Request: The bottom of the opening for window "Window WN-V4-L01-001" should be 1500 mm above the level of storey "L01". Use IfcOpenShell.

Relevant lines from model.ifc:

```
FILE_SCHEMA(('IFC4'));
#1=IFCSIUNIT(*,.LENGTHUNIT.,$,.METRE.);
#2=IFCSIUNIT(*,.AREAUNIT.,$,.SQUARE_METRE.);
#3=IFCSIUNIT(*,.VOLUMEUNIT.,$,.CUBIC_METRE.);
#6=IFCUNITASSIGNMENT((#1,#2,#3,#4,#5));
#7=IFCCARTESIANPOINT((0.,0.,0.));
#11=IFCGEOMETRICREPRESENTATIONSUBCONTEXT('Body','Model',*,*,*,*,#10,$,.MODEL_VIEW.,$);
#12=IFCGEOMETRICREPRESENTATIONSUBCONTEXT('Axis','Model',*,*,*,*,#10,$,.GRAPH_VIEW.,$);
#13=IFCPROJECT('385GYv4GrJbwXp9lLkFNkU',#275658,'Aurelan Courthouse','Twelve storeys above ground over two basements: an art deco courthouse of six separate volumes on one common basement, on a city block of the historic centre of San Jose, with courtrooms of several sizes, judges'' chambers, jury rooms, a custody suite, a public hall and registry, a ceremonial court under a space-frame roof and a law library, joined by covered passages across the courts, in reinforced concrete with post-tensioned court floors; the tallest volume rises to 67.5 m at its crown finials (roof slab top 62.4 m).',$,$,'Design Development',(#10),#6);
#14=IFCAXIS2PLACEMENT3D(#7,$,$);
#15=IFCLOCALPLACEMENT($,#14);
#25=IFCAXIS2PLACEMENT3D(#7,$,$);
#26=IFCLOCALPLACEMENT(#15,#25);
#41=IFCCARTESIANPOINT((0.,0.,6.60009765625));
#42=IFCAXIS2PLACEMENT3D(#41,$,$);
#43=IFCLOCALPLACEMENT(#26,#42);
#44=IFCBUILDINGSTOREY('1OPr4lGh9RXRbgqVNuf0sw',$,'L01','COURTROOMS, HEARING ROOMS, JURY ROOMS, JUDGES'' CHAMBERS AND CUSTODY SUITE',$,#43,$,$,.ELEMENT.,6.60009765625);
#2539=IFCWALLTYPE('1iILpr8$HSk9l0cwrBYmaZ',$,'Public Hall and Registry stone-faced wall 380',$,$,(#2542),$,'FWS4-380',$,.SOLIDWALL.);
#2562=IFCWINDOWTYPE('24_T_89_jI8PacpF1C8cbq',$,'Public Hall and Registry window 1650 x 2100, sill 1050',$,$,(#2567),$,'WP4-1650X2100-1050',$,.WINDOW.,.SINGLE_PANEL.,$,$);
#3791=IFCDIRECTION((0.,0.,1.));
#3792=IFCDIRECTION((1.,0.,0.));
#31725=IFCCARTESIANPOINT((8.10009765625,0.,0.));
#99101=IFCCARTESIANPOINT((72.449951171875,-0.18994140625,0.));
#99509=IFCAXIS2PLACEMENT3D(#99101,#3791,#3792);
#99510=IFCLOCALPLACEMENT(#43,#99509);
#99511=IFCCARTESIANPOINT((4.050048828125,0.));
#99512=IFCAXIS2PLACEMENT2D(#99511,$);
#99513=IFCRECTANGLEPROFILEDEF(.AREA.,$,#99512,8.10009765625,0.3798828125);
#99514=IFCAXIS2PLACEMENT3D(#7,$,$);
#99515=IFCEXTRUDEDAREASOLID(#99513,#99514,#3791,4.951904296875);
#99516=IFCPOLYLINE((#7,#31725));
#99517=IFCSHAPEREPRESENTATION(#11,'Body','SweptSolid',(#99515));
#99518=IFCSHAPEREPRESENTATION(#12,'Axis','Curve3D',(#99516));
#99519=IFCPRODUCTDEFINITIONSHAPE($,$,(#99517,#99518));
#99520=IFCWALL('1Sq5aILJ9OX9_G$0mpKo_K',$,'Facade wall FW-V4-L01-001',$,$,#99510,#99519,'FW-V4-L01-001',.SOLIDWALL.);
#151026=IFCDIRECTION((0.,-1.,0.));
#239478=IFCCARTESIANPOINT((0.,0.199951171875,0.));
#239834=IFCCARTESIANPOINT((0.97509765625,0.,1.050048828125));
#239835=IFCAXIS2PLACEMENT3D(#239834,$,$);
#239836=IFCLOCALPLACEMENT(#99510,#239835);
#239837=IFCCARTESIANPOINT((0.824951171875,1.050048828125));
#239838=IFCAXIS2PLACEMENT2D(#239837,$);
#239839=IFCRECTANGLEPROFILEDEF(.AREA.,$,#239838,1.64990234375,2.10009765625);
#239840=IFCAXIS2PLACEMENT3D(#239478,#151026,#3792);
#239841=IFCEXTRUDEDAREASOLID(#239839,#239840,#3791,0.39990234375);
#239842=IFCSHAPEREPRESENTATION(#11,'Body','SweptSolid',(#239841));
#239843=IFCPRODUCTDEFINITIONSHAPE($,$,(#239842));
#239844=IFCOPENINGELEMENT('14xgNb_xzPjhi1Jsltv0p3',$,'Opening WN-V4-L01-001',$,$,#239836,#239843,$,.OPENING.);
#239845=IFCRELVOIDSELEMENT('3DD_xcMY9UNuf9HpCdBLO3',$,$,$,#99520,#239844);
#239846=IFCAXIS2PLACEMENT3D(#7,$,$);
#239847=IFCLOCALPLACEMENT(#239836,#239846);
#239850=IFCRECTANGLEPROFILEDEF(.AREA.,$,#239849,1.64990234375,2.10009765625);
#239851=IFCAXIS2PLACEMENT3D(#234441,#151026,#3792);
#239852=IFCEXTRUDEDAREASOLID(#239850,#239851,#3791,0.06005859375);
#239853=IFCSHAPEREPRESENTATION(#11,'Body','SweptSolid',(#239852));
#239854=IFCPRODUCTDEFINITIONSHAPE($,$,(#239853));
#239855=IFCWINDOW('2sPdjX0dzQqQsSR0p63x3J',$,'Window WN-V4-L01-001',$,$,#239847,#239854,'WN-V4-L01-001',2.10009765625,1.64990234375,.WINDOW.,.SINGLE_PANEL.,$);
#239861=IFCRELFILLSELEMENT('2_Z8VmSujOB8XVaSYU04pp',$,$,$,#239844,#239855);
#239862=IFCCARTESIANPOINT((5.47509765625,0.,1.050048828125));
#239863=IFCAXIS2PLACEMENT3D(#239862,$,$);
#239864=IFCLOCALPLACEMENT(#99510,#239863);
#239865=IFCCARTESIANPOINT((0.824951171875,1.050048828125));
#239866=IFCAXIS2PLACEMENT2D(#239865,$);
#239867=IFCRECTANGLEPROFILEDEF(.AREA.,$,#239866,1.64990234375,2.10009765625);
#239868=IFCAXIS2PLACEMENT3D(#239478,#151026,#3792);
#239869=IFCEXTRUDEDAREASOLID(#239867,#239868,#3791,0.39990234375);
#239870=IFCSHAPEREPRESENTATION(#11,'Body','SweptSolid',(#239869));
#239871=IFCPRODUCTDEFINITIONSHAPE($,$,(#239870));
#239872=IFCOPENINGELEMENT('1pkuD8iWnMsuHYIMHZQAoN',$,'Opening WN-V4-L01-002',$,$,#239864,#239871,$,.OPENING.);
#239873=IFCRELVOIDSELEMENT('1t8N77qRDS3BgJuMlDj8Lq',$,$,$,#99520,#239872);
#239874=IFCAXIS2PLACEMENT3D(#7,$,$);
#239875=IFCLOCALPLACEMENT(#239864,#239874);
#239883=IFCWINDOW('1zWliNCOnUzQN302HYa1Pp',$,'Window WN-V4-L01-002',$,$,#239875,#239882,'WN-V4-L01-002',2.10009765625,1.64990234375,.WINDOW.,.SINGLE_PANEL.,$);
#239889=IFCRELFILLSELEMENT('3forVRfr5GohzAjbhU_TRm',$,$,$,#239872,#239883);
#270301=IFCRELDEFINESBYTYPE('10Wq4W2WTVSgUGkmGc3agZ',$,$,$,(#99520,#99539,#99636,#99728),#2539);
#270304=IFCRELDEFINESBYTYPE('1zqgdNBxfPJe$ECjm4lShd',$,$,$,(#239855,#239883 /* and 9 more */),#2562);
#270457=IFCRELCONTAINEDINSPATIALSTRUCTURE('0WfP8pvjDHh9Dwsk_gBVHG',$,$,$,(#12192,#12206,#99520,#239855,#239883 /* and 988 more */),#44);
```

```python
import numpy as np
import ifcopenshell
import ifcopenshell.api.geometry
import ifcopenshell.geom
import ifcopenshell.util.element
import ifcopenshell.util.placement
import ifcopenshell.util.shape
import ifcopenshell.util.unit

model = ifcopenshell.open("model.ifc")
unit_scale = ifcopenshell.util.unit.calculate_unit_scale(model)

window = model.by_guid("2sPdjX0dzQqQsSR0p63x3J")
opening = window.FillsVoids[0].RelatingOpeningElement
storey = ifcopenshell.util.element.get_container(window, ifc_class="IfcBuildingStorey")
level = ifcopenshell.util.placement.get_local_placement(storey.ObjectPlacement)[2, 3]

# The opening's origin need not be at the sill, so measure its lowest point.
shape = ifcopenshell.geom.create_shape(ifcopenshell.geom.settings(), opening)
bottom = ifcopenshell.util.shape.get_shape_bottom_elevation(shape, shape.geometry) / unit_scale
dz = level + 1.5 - bottom

shift = np.array([0.0, 0.0, dz])
# The window is placed relative to its opening, so it follows when the opening moves.
matrix = ifcopenshell.util.placement.get_local_placement(opening.ObjectPlacement)
matrix[:3, 3] += shift
ifcopenshell.api.geometry.edit_object_placement(
    model, product=opening, matrix=matrix, is_si=False, should_transform_children=True
)

print(f"moved by {dz * unit_scale:+.3f} m")

model.write("model_edited.ifc")
```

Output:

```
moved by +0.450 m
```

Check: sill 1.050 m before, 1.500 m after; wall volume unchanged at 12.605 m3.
